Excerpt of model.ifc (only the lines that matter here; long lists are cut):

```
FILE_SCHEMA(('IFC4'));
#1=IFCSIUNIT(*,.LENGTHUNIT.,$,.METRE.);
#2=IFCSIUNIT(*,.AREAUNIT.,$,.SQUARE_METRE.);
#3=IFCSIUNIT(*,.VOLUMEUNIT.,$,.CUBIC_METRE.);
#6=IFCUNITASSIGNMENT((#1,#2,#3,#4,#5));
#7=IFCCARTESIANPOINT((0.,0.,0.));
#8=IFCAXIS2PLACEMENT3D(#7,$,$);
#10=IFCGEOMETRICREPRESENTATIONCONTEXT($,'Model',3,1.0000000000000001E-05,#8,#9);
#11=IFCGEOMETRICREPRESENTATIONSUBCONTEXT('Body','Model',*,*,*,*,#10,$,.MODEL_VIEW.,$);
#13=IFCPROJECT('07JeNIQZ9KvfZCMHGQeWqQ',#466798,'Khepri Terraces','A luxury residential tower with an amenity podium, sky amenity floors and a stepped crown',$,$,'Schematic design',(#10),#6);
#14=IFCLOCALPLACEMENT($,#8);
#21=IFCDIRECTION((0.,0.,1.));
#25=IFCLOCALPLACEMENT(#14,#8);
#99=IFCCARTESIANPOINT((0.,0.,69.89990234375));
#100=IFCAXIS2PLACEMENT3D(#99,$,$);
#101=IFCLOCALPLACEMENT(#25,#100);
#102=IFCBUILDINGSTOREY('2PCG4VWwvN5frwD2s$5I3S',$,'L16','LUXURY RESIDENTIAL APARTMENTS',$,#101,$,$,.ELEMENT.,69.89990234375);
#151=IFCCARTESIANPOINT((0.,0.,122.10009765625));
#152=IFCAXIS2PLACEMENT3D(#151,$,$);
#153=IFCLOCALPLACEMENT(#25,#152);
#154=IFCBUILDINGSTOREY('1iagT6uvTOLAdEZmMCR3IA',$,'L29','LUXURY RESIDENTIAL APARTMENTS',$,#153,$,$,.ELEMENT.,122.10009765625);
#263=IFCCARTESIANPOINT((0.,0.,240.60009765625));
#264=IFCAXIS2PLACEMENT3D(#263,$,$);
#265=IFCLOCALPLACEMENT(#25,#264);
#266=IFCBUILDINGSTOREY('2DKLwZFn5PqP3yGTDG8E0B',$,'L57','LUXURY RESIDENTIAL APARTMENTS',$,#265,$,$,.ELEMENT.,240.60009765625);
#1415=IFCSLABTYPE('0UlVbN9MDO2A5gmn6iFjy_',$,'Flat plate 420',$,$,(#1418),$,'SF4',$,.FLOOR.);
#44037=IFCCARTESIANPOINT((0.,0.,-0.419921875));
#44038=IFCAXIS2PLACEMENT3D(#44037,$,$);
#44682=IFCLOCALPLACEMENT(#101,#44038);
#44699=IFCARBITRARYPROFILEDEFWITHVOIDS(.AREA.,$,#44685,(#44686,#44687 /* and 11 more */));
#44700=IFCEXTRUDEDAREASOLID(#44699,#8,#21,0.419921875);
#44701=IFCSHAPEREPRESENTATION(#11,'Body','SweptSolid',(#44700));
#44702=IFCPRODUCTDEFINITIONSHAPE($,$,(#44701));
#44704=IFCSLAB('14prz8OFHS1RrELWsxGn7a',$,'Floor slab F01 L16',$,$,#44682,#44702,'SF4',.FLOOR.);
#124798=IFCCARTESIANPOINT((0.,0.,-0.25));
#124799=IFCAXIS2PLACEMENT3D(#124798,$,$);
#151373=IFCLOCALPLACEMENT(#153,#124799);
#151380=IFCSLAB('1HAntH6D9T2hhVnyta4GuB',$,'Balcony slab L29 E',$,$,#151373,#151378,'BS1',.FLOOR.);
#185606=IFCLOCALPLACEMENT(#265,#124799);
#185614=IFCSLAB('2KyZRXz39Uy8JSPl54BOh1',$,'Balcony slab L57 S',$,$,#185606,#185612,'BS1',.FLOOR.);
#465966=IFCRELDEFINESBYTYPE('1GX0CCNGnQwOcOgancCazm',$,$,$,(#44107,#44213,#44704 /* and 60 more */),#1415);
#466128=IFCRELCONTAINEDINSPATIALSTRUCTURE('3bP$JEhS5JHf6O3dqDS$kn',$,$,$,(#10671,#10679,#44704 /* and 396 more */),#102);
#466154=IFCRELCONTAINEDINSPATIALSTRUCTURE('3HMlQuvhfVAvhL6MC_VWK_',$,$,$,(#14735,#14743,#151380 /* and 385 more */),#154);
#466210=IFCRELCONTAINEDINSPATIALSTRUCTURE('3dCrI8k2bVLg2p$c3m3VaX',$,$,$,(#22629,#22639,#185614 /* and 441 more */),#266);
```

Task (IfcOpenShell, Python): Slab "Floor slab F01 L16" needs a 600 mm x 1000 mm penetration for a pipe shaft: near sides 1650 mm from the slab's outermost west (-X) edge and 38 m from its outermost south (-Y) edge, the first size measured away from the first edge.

```python
import numpy as np
import ifcopenshell
import ifcopenshell.api.feature
import ifcopenshell.api.geometry
import ifcopenshell.api.root
import ifcopenshell.geom
import ifcopenshell.util.placement
import ifcopenshell.util.representation
import ifcopenshell.util.shape
import ifcopenshell.util.unit

model = ifcopenshell.open("model.ifc")
unit_scale = ifcopenshell.util.unit.calculate_unit_scale(model)
settings = ifcopenshell.geom.settings()


def volume(element):
    """Net volume in cubic metres, openings subtracted."""
    shape = ifcopenshell.geom.create_shape(settings, element)
    return ifcopenshell.util.shape.get_volume(shape.geometry)


slab = model.by_guid("14prz8OFHS1RrELWsxGn7a")
before = volume(slab)

# Extent in the slab's own axes, in metres. The edges named are its -X and -Y sides.
slab_shape = ifcopenshell.geom.create_shape(settings, slab)
vertices = ifcopenshell.util.shape.get_vertices(slab_shape.geometry)
x_min, y_min, bottom = vertices.min(axis=0)
top = vertices[:, 2].max()

opening = ifcopenshell.api.root.create_entity(model, ifc_class="IfcOpeningElement", name="Pipe shaft opening", predefined_type="OPENING")
context = ifcopenshell.util.representation.get_context(model, "Model", "Body", "MODEL_VIEW")
width, depth = 0.6, 1
outline = [(0.0, 0.0), (width, 0.0), (width, depth), (0.0, depth), (0.0, 0.0)]
# Overshoot both faces by 50 mm so the cut is clean.
shape = ifcopenshell.api.geometry.add_slab_representation(
    model, context=context, depth=top - bottom + 0.1, polyline=outline
)
ifcopenshell.api.geometry.assign_representation(model, product=opening, representation=shape)

matrix = ifcopenshell.util.placement.get_local_placement(slab.ObjectPlacement)
matrix[:, 3] = matrix @ np.append(np.array([x_min + 1.65, y_min + 38, bottom - 0.05]) / unit_scale, 1.0)
ifcopenshell.api.geometry.edit_object_placement(model, product=opening, matrix=matrix, is_si=False)
ifcopenshell.api.feature.add_feature(model, feature=opening, element=slab)

after = volume(slab)

print(f"slab volume {before:.3f} -> {after:.3f} m3")

model.write("model_v2.ifc")
```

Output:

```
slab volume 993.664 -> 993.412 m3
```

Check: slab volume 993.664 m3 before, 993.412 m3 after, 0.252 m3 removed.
